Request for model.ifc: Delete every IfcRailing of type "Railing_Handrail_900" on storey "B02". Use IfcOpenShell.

First a look at what the model holds.

```python
import ifcopenshell
import ifcopenshell.util.element

model = ifcopenshell.open("model.ifc")
print(model.schema)
storey = next(s for s in model.by_type("IfcBuildingStorey") if s.Name == "B02")
railings = [e for e in ifcopenshell.util.element.get_decomposition(storey) if e.is_a("IfcRailing")]
seen = {}
for e in railings:
    element_type = ifcopenshell.util.element.get_type(e)
    name = element_type.Name if element_type not in (None, e) else None
    seen[name] = seen.get(name, 0) + 1
for name, count in sorted(seen.items(), key=str):
    print(count, "x", name)
```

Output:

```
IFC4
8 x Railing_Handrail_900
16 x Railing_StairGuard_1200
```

```python
import ifcopenshell
import ifcopenshell.api.root
import ifcopenshell.util.element

model = ifcopenshell.open("model.ifc")

storey = next(s for s in model.by_type("IfcBuildingStorey") if s.Name == "B02")
railings = [e for e in ifcopenshell.util.element.get_decomposition(storey) if e.is_a("IfcRailing")]
targets = [e for e in railings if (t := ifcopenshell.util.element.get_type(e)) not in (None, e) and t.Name == "Railing_Handrail_900"]

for e in targets:
    ifcopenshell.api.root.remove_product(model, product=e)
print(len(targets), "removed")

model.write("model_rev.ifc")
```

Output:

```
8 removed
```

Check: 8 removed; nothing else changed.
